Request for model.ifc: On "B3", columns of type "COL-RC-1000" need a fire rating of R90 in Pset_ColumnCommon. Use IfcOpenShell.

First a look at what the model holds.

```python
import ifcopenshell
import ifcopenshell.util.element

model = ifcopenshell.open("model.ifc")
print(model.schema)
storey = next(s for s in model.by_type("IfcBuildingStorey") if s.Name == "B3")
columns = [e for e in ifcopenshell.util.element.get_decomposition(storey) if e.is_a("IfcColumn")]
seen = {}
for e in columns:
    element_type = ifcopenshell.util.element.get_type(e)
    key = (element_type.Name if element_type != e and element_type else None, ifcopenshell.util.element.get_pset(e, "Pset_ColumnCommon", "FireRating"))
    seen[key] = seen.get(key, 0) + 1
for (name, value), count in sorted(seen.items(), key=str):
    print(count, "x", name, "|", value)
```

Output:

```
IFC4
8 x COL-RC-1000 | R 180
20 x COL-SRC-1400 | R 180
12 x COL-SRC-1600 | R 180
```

```python
import ifcopenshell
import ifcopenshell.api.pset
import ifcopenshell.util.element

model = ifcopenshell.open("model.ifc")

storey = next(s for s in model.by_type("IfcBuildingStorey") if s.Name == "B3")
columns = [e for e in ifcopenshell.util.element.get_decomposition(storey) if e.is_a("IfcColumn")]

count = 0
for e in columns:
    element_type = ifcopenshell.util.element.get_type(e)
    if element_type in (None, e) or element_type.Name != "COL-RC-1000":
        continue
    found = ifcopenshell.util.element.get_pset(e, "Pset_ColumnCommon", should_inherit=False)
    if found:
        pset = model.by_id(found["id"])
        if len(ifcopenshell.util.element.get_elements_by_pset(pset)) > 1:
            pset = ifcopenshell.api.pset.unshare_pset(model, products=[e], pset=pset)[0]
    else:
        pset = ifcopenshell.api.pset.add_pset(model, product=e, name="Pset_ColumnCommon")
    ifcopenshell.api.pset.edit_pset(model, pset=pset, properties={"FireRating": "R90"})
    count += 1

print(count, "columns updated")

model.write("model_rev.ifc")
```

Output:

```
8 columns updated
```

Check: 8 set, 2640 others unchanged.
